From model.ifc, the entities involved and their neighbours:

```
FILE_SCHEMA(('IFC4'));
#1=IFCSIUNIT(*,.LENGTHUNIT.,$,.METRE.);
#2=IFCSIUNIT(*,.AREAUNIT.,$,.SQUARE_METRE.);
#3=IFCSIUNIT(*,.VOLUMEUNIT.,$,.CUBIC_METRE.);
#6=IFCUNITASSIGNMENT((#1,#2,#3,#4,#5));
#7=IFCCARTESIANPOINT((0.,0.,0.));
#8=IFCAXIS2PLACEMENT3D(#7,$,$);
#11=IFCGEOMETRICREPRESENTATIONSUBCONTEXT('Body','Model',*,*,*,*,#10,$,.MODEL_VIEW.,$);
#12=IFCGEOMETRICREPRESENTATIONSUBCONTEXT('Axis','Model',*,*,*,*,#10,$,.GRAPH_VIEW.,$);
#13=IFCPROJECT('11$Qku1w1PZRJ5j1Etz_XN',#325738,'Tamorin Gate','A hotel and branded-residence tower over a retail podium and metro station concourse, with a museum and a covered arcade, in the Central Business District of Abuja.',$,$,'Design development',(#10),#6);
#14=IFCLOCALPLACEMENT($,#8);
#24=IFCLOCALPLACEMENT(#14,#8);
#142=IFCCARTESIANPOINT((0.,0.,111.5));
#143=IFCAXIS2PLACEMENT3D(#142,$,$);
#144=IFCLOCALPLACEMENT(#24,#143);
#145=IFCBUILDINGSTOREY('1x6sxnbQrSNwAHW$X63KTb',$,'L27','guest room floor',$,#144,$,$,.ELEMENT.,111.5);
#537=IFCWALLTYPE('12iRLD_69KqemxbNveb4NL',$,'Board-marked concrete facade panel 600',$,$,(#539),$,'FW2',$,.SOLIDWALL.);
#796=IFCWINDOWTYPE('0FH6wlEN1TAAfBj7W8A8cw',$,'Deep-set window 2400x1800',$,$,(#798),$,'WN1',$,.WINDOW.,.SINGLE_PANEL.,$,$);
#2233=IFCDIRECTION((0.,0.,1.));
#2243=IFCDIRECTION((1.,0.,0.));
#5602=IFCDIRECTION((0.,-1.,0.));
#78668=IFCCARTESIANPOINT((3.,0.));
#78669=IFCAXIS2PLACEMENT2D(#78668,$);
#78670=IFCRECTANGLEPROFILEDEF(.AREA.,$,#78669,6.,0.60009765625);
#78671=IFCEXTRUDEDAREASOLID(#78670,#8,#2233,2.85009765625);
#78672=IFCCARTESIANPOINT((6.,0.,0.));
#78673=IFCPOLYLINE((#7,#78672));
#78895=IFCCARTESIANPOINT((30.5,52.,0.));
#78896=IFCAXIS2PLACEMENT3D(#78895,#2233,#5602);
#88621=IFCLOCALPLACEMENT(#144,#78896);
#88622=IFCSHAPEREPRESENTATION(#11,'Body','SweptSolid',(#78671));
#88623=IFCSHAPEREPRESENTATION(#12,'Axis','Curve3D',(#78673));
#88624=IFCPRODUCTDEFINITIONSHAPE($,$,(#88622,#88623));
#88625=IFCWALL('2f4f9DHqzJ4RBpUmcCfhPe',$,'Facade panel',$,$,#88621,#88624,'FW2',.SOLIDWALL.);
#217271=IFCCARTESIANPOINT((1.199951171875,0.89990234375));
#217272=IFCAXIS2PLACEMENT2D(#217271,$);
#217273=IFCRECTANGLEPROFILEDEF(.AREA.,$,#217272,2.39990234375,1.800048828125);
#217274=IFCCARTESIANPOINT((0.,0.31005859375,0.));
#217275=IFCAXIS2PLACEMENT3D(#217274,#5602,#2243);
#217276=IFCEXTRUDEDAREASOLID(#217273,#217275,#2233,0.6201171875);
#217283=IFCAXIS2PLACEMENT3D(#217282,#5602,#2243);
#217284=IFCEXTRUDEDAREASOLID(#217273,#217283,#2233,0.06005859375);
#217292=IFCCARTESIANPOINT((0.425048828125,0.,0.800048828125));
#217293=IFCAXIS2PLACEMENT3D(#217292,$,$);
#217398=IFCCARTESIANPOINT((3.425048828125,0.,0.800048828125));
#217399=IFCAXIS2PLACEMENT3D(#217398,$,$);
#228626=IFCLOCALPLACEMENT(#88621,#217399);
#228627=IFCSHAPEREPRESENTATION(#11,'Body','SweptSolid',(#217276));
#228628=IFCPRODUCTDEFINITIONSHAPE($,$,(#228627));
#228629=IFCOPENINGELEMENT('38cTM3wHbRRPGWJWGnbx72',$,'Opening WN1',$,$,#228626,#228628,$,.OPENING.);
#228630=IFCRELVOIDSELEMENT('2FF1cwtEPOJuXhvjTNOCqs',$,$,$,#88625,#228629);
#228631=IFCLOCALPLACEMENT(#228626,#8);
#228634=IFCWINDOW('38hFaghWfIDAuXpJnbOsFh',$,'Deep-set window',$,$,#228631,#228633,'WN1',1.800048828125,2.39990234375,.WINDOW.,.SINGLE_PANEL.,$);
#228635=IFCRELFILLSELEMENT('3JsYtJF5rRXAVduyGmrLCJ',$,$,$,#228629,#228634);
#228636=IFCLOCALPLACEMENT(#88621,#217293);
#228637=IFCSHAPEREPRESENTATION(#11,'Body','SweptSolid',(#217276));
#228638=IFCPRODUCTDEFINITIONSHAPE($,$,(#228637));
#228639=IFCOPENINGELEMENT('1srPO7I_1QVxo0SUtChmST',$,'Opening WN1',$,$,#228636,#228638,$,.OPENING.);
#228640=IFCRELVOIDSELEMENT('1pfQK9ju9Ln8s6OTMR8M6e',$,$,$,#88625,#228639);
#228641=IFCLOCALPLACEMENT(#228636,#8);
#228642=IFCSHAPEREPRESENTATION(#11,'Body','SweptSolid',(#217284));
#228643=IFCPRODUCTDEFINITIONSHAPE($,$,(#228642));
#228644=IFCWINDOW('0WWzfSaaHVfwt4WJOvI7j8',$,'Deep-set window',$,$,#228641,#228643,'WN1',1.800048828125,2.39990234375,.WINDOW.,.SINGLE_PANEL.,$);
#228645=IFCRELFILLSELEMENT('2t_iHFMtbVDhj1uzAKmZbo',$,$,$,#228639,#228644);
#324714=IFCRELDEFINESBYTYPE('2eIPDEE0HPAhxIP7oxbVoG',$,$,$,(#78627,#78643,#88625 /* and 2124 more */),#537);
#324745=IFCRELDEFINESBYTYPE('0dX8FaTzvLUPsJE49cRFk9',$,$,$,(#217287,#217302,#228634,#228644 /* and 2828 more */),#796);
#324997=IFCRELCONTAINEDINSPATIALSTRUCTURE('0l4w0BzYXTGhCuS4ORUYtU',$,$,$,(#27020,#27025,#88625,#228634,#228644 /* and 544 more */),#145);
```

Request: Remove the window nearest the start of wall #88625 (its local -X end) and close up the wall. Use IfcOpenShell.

```python
import ifcopenshell
import ifcopenshell.api.feature
import ifcopenshell.api.root
import ifcopenshell.geom
import ifcopenshell.util.shape

model = ifcopenshell.open("model.ifc")
settings = ifcopenshell.geom.settings()


def volume(element):
    """Net volume in cubic metres, openings subtracted."""
    shape = ifcopenshell.geom.create_shape(settings, element)
    return ifcopenshell.util.shape.get_volume(shape.geometry)


window = model.by_guid("0WWzfSaaHVfwt4WJOvI7j8")
opening = window.FillsVoids[0].RelatingOpeningElement
wall = opening.VoidsElements[0].RelatingBuildingElement
before = volume(wall)

ifcopenshell.api.root.remove_product(model, product=window)
ifcopenshell.api.feature.remove_feature(model, feature=opening)

after = volume(wall)

print(f"wall volume {before:.3f} -> {after:.3f} m3")

model.write("model-out.ifc")
```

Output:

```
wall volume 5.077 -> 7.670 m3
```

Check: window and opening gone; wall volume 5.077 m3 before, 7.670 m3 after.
